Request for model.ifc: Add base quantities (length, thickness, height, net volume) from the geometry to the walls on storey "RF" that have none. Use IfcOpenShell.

First a look at what the model holds.

```python
import ifcopenshell
import ifcopenshell.util.element
import ifcopenshell.util.unit

model = ifcopenshell.open("model.ifc")
print(model.schema)
for unit_type in ("LENGTHUNIT", "AREAUNIT", "VOLUMEUNIT"):
    print(unit_type, ifcopenshell.util.unit.calculate_unit_scale(model, unit_type))
storey = next(s for s in model.by_type("IfcBuildingStorey") if s.Name == "RF")
walls = [e for e in ifcopenshell.util.element.get_decomposition(storey) if e.is_a("IfcWall")]
for e in sorted(walls, key=lambda e: e.id()):
    print(e.id(), e.is_a(), e.Name, list(ifcopenshell.util.element.get_psets(e, qtos_only=True)), sep=" | ")
```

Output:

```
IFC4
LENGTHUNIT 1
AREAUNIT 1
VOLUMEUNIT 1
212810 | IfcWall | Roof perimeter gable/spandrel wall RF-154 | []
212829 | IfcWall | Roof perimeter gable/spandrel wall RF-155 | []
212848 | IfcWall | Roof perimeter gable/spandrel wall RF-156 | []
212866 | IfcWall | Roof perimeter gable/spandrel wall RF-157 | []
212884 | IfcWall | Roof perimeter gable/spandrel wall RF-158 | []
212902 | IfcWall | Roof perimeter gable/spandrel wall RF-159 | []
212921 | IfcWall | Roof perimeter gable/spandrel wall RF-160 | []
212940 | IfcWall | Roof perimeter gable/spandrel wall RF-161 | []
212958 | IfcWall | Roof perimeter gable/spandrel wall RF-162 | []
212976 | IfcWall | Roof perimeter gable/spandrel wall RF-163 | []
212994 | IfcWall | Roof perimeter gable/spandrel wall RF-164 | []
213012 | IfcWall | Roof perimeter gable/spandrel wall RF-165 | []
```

```python
import ifcopenshell
import ifcopenshell.api.pset
import ifcopenshell.geom
import ifcopenshell.util.element
import ifcopenshell.util.shape
import ifcopenshell.util.unit

model = ifcopenshell.open("model.ifc")
unit_scale = ifcopenshell.util.unit.calculate_unit_scale(model)
volume_scale = ifcopenshell.util.unit.calculate_unit_scale(model, "VOLUMEUNIT")
settings = ifcopenshell.geom.settings()

storey = next(s for s in model.by_type("IfcBuildingStorey") if s.Name == "RF")
walls = [e for e in ifcopenshell.util.element.get_decomposition(storey) if e.is_a("IfcWall")]

for e in sorted(walls, key=lambda e: e.id()):
    if ifcopenshell.util.element.get_psets(e, qtos_only=True, should_inherit=False):
        continue
    # Geometry comes back in metres, in the element's own axes.
    shape = ifcopenshell.geom.create_shape(settings, e)
    values = {
        "Length": ifcopenshell.util.shape.get_x(shape.geometry) / unit_scale,
        "Width": ifcopenshell.util.shape.get_y(shape.geometry) / unit_scale,
        "Height": ifcopenshell.util.shape.get_z(shape.geometry) / unit_scale,
        "NetVolume": ifcopenshell.util.shape.get_volume(shape.geometry) / volume_scale,
    }
    qto = ifcopenshell.api.pset.add_qto(model, product=e, name="Qto_WallBaseQuantities")
    ifcopenshell.api.pset.edit_qto(model, qto=qto, properties=values)
    print(e.id(), {k: round(v, 3) for k, v in values.items()})

model.write("model_v2.ifc")
```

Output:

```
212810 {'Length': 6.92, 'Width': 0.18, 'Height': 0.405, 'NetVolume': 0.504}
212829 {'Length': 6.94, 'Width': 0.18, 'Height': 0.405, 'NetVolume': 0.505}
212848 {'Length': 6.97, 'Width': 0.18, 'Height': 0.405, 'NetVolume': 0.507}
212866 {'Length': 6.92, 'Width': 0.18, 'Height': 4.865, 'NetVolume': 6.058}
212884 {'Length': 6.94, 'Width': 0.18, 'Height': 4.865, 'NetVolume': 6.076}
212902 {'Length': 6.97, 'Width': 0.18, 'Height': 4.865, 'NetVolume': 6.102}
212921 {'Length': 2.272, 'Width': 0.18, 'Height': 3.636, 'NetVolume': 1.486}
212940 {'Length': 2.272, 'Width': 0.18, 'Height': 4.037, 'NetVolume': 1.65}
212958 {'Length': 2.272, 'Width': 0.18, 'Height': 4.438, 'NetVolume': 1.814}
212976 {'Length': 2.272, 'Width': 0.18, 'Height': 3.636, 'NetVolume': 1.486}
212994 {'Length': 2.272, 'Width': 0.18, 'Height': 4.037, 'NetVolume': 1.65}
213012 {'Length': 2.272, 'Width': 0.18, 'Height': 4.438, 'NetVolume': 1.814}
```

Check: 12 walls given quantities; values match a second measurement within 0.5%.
